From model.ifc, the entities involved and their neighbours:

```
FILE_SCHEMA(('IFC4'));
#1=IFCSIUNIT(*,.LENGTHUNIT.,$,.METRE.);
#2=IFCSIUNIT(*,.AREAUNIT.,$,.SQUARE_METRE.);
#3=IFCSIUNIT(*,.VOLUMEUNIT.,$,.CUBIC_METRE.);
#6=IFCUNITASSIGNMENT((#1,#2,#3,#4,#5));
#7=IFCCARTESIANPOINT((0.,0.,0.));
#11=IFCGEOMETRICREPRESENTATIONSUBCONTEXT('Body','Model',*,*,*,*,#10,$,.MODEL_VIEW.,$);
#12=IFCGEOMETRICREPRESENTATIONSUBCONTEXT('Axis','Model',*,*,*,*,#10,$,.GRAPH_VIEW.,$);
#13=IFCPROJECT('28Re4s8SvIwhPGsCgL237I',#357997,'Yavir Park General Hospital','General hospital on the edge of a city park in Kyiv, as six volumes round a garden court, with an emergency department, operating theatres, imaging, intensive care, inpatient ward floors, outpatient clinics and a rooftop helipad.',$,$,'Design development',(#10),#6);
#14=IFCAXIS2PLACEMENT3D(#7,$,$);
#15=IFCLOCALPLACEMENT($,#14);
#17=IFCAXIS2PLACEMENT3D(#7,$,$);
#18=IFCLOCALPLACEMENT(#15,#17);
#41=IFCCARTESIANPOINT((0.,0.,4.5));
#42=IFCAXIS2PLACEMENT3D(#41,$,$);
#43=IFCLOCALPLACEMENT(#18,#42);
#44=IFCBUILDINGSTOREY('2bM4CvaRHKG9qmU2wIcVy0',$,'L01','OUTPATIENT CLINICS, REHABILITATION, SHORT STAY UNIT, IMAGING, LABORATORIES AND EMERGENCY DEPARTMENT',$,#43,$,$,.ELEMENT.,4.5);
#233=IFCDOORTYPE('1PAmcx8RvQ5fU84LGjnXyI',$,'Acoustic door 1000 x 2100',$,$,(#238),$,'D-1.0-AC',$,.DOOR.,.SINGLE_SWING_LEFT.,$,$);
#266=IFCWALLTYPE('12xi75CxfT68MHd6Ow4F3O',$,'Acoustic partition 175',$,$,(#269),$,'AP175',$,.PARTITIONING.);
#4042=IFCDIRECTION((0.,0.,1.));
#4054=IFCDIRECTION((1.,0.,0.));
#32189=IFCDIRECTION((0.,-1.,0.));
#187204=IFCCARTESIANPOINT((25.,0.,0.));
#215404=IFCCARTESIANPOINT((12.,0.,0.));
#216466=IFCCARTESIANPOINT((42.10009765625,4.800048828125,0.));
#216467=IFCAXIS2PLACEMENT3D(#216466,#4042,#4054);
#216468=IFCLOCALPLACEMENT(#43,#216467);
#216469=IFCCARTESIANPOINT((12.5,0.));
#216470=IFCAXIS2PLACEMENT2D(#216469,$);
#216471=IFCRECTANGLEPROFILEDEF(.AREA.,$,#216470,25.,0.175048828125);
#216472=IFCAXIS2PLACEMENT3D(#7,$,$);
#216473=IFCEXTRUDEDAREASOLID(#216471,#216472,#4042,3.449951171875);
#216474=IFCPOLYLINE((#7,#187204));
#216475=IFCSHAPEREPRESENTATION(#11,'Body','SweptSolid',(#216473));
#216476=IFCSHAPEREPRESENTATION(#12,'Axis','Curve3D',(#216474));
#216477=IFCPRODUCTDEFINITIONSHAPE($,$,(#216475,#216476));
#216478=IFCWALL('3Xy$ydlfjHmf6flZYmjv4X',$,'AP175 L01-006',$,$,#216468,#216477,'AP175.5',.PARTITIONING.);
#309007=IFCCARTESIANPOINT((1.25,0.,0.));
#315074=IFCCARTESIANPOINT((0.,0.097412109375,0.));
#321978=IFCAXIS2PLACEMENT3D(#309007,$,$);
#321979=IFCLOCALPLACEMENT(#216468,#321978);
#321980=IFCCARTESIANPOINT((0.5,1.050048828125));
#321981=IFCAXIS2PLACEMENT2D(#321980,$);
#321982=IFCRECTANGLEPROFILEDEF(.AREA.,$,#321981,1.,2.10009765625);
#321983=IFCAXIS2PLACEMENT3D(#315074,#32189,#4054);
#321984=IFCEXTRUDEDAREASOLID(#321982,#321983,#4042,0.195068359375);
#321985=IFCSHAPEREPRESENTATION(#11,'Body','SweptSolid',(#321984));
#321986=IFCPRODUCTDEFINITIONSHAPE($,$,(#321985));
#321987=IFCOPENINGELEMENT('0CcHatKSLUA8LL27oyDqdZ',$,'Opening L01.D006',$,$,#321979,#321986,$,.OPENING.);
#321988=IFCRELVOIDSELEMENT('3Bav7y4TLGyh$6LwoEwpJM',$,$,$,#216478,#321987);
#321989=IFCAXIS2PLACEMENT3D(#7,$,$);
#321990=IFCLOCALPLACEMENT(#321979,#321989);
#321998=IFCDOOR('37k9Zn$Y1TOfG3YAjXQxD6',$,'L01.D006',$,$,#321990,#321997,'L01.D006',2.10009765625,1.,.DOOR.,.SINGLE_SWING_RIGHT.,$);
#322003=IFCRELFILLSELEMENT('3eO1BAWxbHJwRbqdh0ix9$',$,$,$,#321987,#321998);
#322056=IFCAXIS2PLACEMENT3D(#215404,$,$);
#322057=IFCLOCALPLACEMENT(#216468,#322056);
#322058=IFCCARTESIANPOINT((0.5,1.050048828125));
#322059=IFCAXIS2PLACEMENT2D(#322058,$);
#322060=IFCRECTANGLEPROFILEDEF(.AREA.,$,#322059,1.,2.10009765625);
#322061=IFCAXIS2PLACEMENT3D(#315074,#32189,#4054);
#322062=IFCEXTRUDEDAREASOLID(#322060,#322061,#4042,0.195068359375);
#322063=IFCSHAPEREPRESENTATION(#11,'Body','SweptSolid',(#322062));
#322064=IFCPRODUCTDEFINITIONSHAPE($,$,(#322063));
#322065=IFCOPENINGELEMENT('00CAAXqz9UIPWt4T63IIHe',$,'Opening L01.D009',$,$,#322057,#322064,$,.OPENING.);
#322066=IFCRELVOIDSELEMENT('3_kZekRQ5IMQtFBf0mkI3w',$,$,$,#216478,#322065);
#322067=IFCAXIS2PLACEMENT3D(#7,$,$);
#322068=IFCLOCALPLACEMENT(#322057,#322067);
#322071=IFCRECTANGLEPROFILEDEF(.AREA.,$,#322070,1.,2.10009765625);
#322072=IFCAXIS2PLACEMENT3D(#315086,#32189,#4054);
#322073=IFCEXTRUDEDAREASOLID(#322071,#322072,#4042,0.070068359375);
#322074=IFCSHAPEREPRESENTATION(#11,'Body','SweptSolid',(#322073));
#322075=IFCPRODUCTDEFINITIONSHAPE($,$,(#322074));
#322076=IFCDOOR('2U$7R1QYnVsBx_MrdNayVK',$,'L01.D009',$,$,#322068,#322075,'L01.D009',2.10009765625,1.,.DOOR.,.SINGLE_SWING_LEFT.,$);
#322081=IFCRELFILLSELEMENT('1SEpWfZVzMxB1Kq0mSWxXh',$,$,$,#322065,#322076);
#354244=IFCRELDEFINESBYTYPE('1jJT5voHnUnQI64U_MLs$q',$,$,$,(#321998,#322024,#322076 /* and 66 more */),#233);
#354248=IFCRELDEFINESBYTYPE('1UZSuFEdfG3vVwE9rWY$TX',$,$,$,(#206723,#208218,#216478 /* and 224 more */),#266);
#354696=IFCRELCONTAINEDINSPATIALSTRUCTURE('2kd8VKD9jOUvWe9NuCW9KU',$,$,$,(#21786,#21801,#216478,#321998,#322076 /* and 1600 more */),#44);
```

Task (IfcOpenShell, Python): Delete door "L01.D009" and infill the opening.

```python
import ifcopenshell
import ifcopenshell.api.feature
import ifcopenshell.api.root
import ifcopenshell.geom
import ifcopenshell.util.shape

model = ifcopenshell.open("model.ifc")
settings = ifcopenshell.geom.settings()


def volume(element):
    """Net volume in cubic metres, openings subtracted."""
    shape = ifcopenshell.geom.create_shape(settings, element)
    return ifcopenshell.util.shape.get_volume(shape.geometry)


door = model.by_id(322076)
opening = door.FillsVoids[0].RelatingOpeningElement
wall = opening.VoidsElements[0].RelatingBuildingElement
before = volume(wall)

ifcopenshell.api.root.remove_product(model, product=door)
ifcopenshell.api.feature.remove_feature(model, feature=opening)

after = volume(wall)

print(f"wall volume {before:.3f} -> {after:.3f} m3")

model.write("model_rev.ifc")
```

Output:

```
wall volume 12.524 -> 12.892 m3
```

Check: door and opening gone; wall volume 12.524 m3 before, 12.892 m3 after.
